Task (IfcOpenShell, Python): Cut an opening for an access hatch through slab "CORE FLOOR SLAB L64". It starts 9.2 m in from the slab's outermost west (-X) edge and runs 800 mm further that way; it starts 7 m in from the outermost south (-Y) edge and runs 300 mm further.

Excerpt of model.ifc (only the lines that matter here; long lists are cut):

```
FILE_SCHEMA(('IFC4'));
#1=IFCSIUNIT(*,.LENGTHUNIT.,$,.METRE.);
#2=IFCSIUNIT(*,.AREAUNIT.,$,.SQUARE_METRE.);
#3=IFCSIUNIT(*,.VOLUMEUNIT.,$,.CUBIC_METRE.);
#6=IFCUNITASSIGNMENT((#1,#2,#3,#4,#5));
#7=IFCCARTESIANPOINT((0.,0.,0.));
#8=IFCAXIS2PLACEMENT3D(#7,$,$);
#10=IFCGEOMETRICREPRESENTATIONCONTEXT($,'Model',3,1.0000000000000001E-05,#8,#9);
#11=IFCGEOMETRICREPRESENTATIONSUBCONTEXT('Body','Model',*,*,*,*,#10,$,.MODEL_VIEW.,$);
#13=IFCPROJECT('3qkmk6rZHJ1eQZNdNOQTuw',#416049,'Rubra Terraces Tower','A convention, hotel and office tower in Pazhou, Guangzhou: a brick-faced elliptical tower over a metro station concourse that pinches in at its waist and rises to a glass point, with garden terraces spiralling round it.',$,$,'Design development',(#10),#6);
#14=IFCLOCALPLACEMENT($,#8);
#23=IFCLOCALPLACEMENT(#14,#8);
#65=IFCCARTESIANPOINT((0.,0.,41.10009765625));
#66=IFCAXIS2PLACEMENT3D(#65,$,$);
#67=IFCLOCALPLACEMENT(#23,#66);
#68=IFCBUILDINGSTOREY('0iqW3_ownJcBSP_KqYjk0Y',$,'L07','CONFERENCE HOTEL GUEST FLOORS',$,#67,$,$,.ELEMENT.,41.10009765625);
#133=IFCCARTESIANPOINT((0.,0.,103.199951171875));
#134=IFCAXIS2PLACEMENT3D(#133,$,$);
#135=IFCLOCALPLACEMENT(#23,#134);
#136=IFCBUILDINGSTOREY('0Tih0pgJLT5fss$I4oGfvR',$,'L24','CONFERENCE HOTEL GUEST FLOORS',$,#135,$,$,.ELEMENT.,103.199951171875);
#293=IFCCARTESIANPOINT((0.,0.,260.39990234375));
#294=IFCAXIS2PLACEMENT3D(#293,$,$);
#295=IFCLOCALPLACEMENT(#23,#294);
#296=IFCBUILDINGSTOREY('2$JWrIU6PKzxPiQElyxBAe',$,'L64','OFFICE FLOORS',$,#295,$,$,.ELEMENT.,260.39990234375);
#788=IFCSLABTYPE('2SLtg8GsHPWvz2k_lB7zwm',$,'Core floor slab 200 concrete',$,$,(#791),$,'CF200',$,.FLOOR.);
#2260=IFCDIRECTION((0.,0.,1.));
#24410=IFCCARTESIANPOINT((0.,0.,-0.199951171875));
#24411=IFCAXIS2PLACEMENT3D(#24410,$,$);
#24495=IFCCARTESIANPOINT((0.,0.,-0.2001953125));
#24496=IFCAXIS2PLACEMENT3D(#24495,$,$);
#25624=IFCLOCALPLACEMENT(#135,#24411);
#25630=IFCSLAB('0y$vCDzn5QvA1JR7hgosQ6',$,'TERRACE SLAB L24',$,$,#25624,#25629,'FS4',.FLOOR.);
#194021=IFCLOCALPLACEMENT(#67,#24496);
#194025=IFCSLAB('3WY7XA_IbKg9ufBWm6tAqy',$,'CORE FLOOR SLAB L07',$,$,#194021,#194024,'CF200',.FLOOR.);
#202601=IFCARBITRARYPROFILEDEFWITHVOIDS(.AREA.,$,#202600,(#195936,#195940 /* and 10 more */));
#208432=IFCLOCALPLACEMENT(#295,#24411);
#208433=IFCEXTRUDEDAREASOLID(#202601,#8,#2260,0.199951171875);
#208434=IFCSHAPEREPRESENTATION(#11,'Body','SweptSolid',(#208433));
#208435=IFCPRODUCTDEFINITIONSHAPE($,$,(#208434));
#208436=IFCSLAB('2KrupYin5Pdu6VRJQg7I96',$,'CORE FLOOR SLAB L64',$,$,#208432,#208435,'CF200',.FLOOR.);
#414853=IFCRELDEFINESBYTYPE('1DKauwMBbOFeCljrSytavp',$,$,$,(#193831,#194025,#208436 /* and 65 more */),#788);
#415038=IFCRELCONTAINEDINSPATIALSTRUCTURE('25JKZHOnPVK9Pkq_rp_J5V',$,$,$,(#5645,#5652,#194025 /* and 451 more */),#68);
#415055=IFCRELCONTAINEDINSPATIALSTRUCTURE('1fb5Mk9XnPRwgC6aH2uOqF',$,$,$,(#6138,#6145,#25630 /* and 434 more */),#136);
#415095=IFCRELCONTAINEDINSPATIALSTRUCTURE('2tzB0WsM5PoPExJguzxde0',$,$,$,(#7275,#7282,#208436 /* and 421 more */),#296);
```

```python
import numpy as np
import ifcopenshell
import ifcopenshell.api.feature
import ifcopenshell.api.geometry
import ifcopenshell.api.root
import ifcopenshell.geom
import ifcopenshell.util.placement
import ifcopenshell.util.representation
import ifcopenshell.util.shape
import ifcopenshell.util.unit

model = ifcopenshell.open("model.ifc")
unit_scale = ifcopenshell.util.unit.calculate_unit_scale(model)
settings = ifcopenshell.geom.settings()


def volume(element):
    """Net volume in cubic metres, openings subtracted."""
    shape = ifcopenshell.geom.create_shape(settings, element)
    return ifcopenshell.util.shape.get_volume(shape.geometry)


slab = model.by_id(208436)
before = volume(slab)

# Extent in the slab's own axes, in metres. The edges named are its -X and -Y sides.
slab_shape = ifcopenshell.geom.create_shape(settings, slab)
vertices = ifcopenshell.util.shape.get_vertices(slab_shape.geometry)
x_min, y_min, bottom = vertices.min(axis=0)
top = vertices[:, 2].max()

opening = ifcopenshell.api.root.create_entity(model, ifc_class="IfcOpeningElement", name="Access hatch opening", predefined_type="OPENING")
context = ifcopenshell.util.representation.get_context(model, "Model", "Body", "MODEL_VIEW")
width, depth = 0.8, 0.3
outline = [(0.0, 0.0), (width, 0.0), (width, depth), (0.0, depth), (0.0, 0.0)]
# Overshoot both faces by 50 mm so the cut is clean.
shape = ifcopenshell.api.geometry.add_slab_representation(
    model, context=context, depth=top - bottom + 0.1, polyline=outline
)
ifcopenshell.api.geometry.assign_representation(model, product=opening, representation=shape)

matrix = ifcopenshell.util.placement.get_local_placement(slab.ObjectPlacement)
matrix[:, 3] = matrix @ np.append(np.array([x_min + 9.2, y_min + 7, bottom - 0.05]) / unit_scale, 1.0)
ifcopenshell.api.geometry.edit_object_placement(model, product=opening, matrix=matrix, is_si=False)
ifcopenshell.api.feature.add_feature(model, feature=opening, element=slab)

after = volume(slab)

print(f"slab volume {before:.3f} -> {after:.3f} m3")

model.write("model_v2.ifc")
```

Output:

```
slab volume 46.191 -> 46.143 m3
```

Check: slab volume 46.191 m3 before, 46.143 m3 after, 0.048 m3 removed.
